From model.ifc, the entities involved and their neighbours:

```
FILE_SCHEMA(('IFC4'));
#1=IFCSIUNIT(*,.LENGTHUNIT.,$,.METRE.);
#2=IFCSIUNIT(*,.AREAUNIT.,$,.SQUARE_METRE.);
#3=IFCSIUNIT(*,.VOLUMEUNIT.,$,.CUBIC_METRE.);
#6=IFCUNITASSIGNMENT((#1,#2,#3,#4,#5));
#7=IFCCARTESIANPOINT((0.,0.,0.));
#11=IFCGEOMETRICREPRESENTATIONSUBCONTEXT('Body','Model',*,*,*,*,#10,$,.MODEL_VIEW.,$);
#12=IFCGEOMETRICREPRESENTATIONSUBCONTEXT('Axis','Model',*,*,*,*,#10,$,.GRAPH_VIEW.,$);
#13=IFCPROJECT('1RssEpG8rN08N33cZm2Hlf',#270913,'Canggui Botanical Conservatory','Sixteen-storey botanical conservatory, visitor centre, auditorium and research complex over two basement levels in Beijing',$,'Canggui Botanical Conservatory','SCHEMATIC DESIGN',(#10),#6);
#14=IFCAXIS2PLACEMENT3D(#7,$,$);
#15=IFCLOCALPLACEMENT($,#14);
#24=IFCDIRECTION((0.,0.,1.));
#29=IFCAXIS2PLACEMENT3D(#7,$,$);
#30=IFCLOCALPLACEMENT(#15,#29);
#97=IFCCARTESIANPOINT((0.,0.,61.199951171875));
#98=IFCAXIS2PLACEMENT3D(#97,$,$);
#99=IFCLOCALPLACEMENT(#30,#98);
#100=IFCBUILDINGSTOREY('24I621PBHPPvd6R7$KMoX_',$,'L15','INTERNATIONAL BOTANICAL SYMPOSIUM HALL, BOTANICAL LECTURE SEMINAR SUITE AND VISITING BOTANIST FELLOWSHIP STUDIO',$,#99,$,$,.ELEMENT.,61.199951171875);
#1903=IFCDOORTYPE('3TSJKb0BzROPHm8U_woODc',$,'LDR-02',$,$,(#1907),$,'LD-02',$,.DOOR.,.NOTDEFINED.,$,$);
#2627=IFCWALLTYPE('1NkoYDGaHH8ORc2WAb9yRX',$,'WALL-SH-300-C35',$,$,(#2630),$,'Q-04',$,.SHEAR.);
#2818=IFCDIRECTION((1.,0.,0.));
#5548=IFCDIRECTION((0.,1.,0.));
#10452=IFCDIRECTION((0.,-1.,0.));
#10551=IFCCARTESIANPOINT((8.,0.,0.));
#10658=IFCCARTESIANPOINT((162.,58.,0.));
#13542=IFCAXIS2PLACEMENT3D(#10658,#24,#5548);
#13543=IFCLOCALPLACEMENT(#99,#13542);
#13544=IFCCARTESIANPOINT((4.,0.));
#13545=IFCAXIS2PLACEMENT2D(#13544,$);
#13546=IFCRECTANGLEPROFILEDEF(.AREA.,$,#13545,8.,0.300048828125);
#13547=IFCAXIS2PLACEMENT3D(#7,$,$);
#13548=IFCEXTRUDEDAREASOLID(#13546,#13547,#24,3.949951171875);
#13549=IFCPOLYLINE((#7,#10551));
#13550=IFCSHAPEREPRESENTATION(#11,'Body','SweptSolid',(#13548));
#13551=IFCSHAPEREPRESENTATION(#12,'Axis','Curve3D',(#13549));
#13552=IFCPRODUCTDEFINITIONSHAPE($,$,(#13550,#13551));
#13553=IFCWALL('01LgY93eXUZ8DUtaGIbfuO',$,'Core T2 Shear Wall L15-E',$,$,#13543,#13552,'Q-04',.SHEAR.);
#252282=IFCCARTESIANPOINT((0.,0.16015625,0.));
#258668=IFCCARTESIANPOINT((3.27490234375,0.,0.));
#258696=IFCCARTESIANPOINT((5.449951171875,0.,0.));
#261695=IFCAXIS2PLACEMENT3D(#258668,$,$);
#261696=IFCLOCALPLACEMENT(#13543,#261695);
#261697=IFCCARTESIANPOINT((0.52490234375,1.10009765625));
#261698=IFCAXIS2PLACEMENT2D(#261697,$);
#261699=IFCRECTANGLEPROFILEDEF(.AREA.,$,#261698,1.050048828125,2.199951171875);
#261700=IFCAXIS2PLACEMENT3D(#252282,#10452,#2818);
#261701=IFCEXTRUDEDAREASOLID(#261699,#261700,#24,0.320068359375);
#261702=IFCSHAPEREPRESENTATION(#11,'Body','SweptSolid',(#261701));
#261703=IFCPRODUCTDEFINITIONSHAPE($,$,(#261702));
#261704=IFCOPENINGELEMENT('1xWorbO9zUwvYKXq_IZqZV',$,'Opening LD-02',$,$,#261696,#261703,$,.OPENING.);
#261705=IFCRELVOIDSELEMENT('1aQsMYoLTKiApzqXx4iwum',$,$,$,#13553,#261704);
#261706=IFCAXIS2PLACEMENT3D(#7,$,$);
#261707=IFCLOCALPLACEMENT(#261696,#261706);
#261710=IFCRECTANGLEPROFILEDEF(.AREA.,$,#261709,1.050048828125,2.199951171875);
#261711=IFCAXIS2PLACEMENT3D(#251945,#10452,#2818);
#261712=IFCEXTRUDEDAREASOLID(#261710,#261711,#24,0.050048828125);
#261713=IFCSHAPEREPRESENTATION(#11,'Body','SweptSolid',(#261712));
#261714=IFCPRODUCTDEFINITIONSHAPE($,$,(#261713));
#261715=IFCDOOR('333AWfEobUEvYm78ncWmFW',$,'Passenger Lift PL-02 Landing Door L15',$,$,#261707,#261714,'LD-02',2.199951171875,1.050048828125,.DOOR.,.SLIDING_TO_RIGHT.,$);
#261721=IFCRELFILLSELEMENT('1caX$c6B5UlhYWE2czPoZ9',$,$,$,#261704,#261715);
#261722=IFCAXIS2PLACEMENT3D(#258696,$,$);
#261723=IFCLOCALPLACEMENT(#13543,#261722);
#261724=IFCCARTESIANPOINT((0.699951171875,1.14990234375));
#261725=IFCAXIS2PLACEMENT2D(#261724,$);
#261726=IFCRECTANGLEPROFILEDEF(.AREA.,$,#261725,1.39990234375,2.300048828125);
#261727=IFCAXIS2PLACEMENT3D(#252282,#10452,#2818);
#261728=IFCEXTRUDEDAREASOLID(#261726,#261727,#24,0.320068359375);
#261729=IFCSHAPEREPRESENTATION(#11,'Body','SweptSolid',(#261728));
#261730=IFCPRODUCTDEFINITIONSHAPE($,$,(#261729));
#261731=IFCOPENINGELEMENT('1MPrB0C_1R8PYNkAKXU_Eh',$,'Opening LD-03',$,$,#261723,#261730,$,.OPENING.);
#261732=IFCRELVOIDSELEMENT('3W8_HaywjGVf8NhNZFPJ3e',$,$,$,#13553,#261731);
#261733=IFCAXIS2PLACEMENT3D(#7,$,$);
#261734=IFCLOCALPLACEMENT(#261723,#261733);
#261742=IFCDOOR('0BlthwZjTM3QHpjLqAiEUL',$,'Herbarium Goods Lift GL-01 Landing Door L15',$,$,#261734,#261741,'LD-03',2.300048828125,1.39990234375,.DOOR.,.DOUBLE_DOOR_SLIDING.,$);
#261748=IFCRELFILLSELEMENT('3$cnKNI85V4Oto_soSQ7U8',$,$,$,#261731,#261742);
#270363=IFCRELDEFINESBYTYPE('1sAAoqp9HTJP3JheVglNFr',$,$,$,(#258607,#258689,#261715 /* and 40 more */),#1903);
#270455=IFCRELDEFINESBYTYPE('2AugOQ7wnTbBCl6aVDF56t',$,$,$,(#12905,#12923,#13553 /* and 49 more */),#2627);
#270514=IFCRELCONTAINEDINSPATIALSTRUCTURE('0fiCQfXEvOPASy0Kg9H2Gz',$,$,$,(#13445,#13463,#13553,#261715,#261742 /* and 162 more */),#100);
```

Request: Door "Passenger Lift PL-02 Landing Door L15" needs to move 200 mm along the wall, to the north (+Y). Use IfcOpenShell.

```python
import ifcopenshell
import ifcopenshell.api.geometry
import ifcopenshell.util.placement

model = ifcopenshell.open("model.ifc")

door = model.by_guid("333AWfEobUEvYm78ncWmFW")
opening = door.FillsVoids[0].RelatingOpeningElement
wall = opening.VoidsElements[0].RelatingBuildingElement

wall_matrix = ifcopenshell.util.placement.get_local_placement(wall.ObjectPlacement)
shift = wall_matrix[:3, 0] * 0.2
before = ifcopenshell.util.placement.get_local_placement(door.ObjectPlacement)[:3, 3].copy()

# The door is placed relative to its opening, so it follows when the opening moves.
matrix = ifcopenshell.util.placement.get_local_placement(opening.ObjectPlacement)
matrix[:3, 3] += shift
ifcopenshell.api.geometry.edit_object_placement(
    model, product=opening, matrix=matrix, is_si=False, should_transform_children=True
)

after = ifcopenshell.util.placement.get_local_placement(door.ObjectPlacement)[:3, 3]
print("door moved by", (after - before).round(3) + 0.0)

model.write("model_updated.ifc")
```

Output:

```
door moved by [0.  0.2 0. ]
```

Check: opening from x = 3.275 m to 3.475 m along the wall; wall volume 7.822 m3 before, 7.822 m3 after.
